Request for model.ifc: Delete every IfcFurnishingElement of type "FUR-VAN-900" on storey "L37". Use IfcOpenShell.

First a look at what the model holds.

```python
import ifcopenshell
import ifcopenshell.util.element

model = ifcopenshell.open("model.ifc")
print(model.schema)
storey = next(s for s in model.by_type("IfcBuildingStorey") if s.Name == "L37")
furniture = [e for e in ifcopenshell.util.element.get_decomposition(storey) if e.is_a("IfcFurnishingElement")]
seen = {}
for e in furniture:
    element_type = ifcopenshell.util.element.get_type(e)
    name = element_type.Name if element_type not in (None, e) else None
    seen[name] = seen.get(name, 0) + 1
for name, count in sorted(seen.items(), key=str):
    print(count, "x", name)
```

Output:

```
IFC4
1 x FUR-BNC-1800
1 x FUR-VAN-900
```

```python
import ifcopenshell
import ifcopenshell.api.root
import ifcopenshell.util.element

model = ifcopenshell.open("model.ifc")

storey = next(s for s in model.by_type("IfcBuildingStorey") if s.Name == "L37")
furniture = [e for e in ifcopenshell.util.element.get_decomposition(storey) if e.is_a("IfcFurnishingElement")]
targets = [e for e in furniture if (t := ifcopenshell.util.element.get_type(e)) not in (None, e) and t.Name == "FUR-VAN-900"]

for e in targets:
    ifcopenshell.api.root.remove_product(model, product=e)
print(len(targets), "removed")

model.write("model_edited.ifc")
```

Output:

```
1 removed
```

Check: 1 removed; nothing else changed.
